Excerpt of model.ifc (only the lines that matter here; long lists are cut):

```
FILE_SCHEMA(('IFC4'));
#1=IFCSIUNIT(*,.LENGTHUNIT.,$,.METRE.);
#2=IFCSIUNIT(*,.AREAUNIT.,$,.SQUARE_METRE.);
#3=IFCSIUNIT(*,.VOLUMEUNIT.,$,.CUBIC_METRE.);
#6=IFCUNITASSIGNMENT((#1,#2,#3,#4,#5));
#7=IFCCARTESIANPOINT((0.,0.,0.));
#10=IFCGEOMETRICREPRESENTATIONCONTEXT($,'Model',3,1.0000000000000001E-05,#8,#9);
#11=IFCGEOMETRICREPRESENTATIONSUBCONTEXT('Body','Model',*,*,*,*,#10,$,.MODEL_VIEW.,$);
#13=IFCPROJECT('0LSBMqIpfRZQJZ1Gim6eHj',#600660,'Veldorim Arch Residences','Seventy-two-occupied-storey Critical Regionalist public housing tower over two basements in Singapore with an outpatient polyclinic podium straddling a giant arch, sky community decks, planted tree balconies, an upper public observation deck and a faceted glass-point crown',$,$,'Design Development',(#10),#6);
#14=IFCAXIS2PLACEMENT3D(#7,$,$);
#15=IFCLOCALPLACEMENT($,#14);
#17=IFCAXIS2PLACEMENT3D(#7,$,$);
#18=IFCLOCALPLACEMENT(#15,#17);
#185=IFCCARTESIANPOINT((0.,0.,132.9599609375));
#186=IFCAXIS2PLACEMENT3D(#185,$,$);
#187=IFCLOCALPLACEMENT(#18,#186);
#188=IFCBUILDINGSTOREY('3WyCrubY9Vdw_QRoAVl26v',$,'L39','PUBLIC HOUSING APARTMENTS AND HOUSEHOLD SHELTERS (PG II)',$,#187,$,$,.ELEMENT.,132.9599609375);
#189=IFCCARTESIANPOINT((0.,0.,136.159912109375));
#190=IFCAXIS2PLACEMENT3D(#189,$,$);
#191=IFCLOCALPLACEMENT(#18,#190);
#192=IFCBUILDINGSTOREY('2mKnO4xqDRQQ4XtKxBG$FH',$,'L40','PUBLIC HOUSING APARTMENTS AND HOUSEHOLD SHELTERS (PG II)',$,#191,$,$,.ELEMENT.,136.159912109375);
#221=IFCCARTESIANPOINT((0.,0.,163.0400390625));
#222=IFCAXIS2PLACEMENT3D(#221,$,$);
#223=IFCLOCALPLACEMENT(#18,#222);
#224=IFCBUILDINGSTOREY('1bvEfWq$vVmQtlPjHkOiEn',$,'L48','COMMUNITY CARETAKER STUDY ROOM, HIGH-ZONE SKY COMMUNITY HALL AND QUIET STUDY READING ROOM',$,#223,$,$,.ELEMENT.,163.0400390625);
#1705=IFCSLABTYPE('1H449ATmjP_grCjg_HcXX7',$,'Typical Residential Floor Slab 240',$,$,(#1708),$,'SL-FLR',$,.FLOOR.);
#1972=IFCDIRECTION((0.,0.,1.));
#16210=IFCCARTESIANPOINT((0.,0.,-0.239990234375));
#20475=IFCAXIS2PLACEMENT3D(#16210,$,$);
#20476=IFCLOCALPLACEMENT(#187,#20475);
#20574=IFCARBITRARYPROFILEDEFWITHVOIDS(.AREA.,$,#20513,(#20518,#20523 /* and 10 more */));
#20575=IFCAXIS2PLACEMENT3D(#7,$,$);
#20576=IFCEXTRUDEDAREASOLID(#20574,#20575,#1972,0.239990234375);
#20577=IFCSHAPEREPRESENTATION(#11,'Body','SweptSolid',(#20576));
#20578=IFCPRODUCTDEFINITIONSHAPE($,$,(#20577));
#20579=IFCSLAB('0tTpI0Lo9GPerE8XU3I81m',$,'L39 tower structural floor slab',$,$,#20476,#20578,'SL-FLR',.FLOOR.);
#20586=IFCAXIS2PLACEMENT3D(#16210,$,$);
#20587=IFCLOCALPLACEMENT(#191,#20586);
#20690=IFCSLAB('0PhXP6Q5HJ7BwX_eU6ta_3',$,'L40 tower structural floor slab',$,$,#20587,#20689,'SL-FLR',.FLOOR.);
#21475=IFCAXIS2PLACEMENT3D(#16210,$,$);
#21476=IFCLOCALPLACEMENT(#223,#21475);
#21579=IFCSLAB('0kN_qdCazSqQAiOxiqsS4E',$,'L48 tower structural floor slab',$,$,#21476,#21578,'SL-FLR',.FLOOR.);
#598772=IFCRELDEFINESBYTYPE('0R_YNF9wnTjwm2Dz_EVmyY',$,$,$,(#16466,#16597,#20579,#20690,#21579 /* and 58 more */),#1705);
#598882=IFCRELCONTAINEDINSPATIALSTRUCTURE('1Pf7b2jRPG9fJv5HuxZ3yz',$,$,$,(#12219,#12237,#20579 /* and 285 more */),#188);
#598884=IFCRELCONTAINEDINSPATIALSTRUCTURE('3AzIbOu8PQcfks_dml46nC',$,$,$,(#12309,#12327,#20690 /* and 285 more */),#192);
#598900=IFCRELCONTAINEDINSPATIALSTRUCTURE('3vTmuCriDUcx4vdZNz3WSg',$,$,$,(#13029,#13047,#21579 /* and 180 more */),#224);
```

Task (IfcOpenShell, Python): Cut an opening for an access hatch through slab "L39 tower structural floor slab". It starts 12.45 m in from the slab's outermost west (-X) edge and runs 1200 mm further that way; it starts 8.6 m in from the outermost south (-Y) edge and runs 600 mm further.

```python
import numpy as np
import ifcopenshell
import ifcopenshell.api.feature
import ifcopenshell.api.geometry
import ifcopenshell.api.root
import ifcopenshell.geom
import ifcopenshell.util.placement
import ifcopenshell.util.representation
import ifcopenshell.util.shape
import ifcopenshell.util.unit

model = ifcopenshell.open("model.ifc")
unit_scale = ifcopenshell.util.unit.calculate_unit_scale(model)
settings = ifcopenshell.geom.settings()


def volume(element):
    """Net volume in cubic metres, openings subtracted."""
    shape = ifcopenshell.geom.create_shape(settings, element)
    return ifcopenshell.util.shape.get_volume(shape.geometry)


slab = model.by_guid("0tTpI0Lo9GPerE8XU3I81m")
before = volume(slab)

# Extent in the slab's own axes, in metres. The edges named are its -X and -Y sides.
slab_shape = ifcopenshell.geom.create_shape(settings, slab)
vertices = ifcopenshell.util.shape.get_vertices(slab_shape.geometry)
x_min, y_min, bottom = vertices.min(axis=0)
top = vertices[:, 2].max()

opening = ifcopenshell.api.root.create_entity(model, ifc_class="IfcOpeningElement", name="Access hatch opening", predefined_type="OPENING")
context = ifcopenshell.util.representation.get_context(model, "Model", "Body", "MODEL_VIEW")
width, depth = 1.2, 0.6
outline = [(0.0, 0.0), (width, 0.0), (width, depth), (0.0, depth), (0.0, 0.0)]
# Overshoot both faces by 50 mm so the cut is clean.
shape = ifcopenshell.api.geometry.add_slab_representation(
    model, context=context, depth=top - bottom + 0.1, polyline=outline
)
ifcopenshell.api.geometry.assign_representation(model, product=opening, representation=shape)

matrix = ifcopenshell.util.placement.get_local_placement(slab.ObjectPlacement)
matrix[:, 3] = matrix @ np.append(np.array([x_min + 12.45, y_min + 8.6, bottom - 0.05]) / unit_scale, 1.0)
ifcopenshell.api.geometry.edit_object_placement(model, product=opening, matrix=matrix, is_si=False)
ifcopenshell.api.feature.add_feature(model, feature=opening, element=slab)

after = volume(slab)

print(f"slab volume {before:.3f} -> {after:.3f} m3")

model.write("model-out.ifc")
```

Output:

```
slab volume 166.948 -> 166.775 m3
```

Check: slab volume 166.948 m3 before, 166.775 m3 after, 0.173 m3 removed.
